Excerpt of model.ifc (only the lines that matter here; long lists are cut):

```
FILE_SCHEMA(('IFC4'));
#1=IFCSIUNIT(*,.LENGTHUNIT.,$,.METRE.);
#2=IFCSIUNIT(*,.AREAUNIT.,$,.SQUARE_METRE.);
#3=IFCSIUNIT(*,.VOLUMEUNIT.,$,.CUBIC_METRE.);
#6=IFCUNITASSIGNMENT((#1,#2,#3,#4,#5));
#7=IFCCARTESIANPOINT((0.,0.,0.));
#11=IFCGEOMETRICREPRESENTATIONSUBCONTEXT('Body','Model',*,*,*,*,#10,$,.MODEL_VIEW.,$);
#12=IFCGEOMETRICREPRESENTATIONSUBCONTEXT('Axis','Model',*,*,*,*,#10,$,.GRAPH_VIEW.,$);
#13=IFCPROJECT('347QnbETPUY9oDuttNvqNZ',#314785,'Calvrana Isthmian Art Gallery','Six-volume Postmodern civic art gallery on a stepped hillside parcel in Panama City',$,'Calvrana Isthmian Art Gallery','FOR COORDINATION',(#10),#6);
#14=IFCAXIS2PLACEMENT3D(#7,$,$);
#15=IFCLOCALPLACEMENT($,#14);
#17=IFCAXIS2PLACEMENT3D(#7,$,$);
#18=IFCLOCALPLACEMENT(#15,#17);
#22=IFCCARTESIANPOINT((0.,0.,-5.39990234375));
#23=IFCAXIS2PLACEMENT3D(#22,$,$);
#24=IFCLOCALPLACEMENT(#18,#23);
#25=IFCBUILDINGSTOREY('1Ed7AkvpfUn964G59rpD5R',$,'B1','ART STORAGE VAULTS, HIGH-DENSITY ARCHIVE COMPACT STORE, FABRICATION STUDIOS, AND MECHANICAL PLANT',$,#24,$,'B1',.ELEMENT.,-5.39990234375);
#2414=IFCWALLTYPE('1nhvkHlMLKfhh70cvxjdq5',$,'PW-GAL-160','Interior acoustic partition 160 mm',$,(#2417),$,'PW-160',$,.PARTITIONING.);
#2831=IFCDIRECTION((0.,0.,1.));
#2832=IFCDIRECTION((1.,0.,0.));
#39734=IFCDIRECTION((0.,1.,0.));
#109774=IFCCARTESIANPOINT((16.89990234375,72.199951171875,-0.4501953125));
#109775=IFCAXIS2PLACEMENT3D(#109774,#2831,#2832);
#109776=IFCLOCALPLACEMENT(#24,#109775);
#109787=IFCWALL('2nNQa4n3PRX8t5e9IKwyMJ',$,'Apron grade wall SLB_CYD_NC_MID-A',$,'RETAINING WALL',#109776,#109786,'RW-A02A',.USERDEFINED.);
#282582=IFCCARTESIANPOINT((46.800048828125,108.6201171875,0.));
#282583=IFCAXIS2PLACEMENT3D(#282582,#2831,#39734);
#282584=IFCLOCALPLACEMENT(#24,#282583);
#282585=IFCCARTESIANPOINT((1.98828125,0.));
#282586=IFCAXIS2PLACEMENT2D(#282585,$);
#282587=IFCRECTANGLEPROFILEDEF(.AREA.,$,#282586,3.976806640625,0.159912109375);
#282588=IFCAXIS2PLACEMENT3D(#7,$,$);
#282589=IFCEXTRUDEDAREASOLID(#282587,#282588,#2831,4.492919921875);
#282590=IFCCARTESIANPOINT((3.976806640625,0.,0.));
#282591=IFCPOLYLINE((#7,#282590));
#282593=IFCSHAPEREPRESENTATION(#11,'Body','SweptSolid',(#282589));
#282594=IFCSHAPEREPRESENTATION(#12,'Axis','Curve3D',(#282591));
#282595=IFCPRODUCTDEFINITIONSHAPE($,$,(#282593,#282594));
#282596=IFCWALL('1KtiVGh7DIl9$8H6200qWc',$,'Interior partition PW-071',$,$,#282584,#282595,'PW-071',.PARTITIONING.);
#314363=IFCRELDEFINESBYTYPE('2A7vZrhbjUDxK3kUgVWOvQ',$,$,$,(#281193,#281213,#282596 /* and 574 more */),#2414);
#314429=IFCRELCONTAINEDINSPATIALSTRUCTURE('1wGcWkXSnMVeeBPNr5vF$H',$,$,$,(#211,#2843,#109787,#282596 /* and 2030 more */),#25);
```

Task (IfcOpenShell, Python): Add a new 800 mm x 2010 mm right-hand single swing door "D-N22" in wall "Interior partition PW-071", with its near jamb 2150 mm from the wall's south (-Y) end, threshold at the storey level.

```python
import numpy as np
import ifcopenshell
import ifcopenshell.api.feature
import ifcopenshell.api.geometry
import ifcopenshell.api.root
import ifcopenshell.api.spatial
import ifcopenshell.geom
import ifcopenshell.util.element
import ifcopenshell.util.placement
import ifcopenshell.util.representation
import ifcopenshell.util.shape
import ifcopenshell.util.unit

model = ifcopenshell.open("model.ifc")
unit_scale = ifcopenshell.util.unit.calculate_unit_scale(model)
settings = ifcopenshell.geom.settings()


def volume(element):
    """Net volume in cubic metres, openings subtracted."""
    shape = ifcopenshell.geom.create_shape(settings, element)
    return ifcopenshell.util.shape.get_volume(shape.geometry)


wall = model.by_id(282596)
storey = ifcopenshell.util.element.get_container(wall, ifc_class="IfcBuildingStorey")
context = ifcopenshell.util.representation.get_context(model, "Model", "Body", "MODEL_VIEW")
before = volume(wall)

width, height, from_end, sill = 0.8, 2.01, 2.15, 0.0  # metres

# The wall runs along its own X axis, and the end named is its -X end.
wall_shape = ifcopenshell.geom.create_shape(settings, wall)
x, y, z = ifcopenshell.util.shape.get_vertices(wall_shape.geometry).T
start = x.min() + from_end
face, thickness = float(y.min()), float(y.max() - y.min())
wall_matrix = ifcopenshell.util.placement.get_local_placement(wall.ObjectPlacement)
level = ifcopenshell.util.placement.get_local_placement(storey.ObjectPlacement)[2, 3]


def in_wall(x, y):
    """Placement at x, y metres in the wall's axes, at sill height."""
    matrix = wall_matrix.copy()
    matrix[:, 3] = wall_matrix @ np.array([x / unit_scale, y / unit_scale, 0.0, 1.0])
    matrix[2, 3] = level + sill / unit_scale
    return matrix


# Opening: a box that overshoots both wall faces by 50 mm.
opening = ifcopenshell.api.root.create_entity(model, ifc_class="IfcOpeningElement", predefined_type="OPENING")
box = ifcopenshell.api.geometry.add_wall_representation(
    model, context=context, length=width, height=height, thickness=thickness + 0.1
)
ifcopenshell.api.geometry.assign_representation(model, product=opening, representation=box)
ifcopenshell.api.geometry.edit_object_placement(model, product=opening, matrix=in_wall(start, face - 0.05), is_si=False)
ifcopenshell.api.feature.add_feature(model, feature=opening, element=wall)

door = ifcopenshell.api.root.create_entity(model, ifc_class="IfcDoor", name="D-N22", predefined_type="DOOR")
door.OverallWidth, door.OverallHeight = width / unit_scale, height / unit_scale
door.OperationType = "SINGLE_SWING_RIGHT"
body = ifcopenshell.api.geometry.add_door_representation(
    model,
    context=context,
    overall_width=door.OverallWidth,
    overall_height=door.OverallHeight,
    operation_type="SINGLE_SWING_RIGHT",
    lining_properties={"LiningDepth": thickness / unit_scale, "ThresholdDepth": thickness / unit_scale},
)
ifcopenshell.api.geometry.assign_representation(model, product=door, representation=body)
ifcopenshell.api.spatial.assign_container(model, products=[door], relating_structure=storey)
ifcopenshell.api.feature.add_filling(model, opening=opening, element=door)

# The lining spans the wall, so the door starts at the wall face.
ifcopenshell.api.geometry.edit_object_placement(model, product=door, matrix=in_wall(start, face), is_si=False)

after = volume(wall)

print(f"wall volume {before:.3f} -> {after:.3f} m3")

model.write("model-out.ifc")
```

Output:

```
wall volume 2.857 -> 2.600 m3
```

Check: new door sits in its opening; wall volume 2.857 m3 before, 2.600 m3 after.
